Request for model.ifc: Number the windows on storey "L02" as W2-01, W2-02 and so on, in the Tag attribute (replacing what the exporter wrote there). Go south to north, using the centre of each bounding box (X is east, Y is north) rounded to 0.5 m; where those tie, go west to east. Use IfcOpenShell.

First a look at what the model holds.

```python
import ifcopenshell
import ifcopenshell.util.element
import ifcopenshell.util.placement

model = ifcopenshell.open("model.ifc")
print(model.schema)
storey = next(s for s in model.by_type("IfcBuildingStorey") if s.Name == "L02")
windows = [e for e in ifcopenshell.util.element.get_decomposition(storey) if e.is_a("IfcWindow")]
for e in sorted(windows, key=lambda e: e.id()):
    origin = ifcopenshell.util.placement.get_local_placement(e.ObjectPlacement)[:3, 3]
    print(e.id(), e.Tag, e.Name, origin.round(2) + 0.0, sep=" | ")
```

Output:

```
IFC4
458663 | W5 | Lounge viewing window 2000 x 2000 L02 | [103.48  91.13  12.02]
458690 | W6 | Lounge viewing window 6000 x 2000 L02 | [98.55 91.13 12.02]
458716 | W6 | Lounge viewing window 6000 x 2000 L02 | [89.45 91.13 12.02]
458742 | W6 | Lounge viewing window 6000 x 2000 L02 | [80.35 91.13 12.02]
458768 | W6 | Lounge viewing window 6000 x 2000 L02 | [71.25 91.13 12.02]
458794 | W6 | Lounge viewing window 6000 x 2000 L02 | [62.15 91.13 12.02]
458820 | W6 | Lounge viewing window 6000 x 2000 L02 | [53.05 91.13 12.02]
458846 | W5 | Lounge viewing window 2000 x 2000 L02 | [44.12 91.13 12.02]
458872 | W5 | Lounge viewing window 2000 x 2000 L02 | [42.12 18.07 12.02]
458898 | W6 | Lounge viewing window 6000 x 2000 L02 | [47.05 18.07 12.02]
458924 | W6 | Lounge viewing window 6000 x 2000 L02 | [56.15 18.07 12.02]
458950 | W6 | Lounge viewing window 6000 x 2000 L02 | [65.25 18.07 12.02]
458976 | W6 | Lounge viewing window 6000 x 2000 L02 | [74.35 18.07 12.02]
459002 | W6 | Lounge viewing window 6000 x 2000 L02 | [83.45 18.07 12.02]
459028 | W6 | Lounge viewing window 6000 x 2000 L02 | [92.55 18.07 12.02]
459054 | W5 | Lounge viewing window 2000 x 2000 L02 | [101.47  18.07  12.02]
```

```python
import ifcopenshell
import ifcopenshell.geom
import ifcopenshell.util.element
import ifcopenshell.util.shape

model = ifcopenshell.open("model.ifc")
settings = ifcopenshell.geom.settings()
settings.set("use-world-coords", True)


def centre(element):
    shape = ifcopenshell.geom.create_shape(settings, element)
    return ifcopenshell.util.shape.get_bbox_centroid(shape.geometry)


storey = next(s for s in model.by_type("IfcBuildingStorey") if s.Name == "L02")
windows = [e for e in ifcopenshell.util.element.get_decomposition(storey) if e.is_a("IfcWindow")]

# Insertion points can sit at a corner or the storey origin, so sort by the geometry (in metres).
centres = {e: centre(e) for e in windows}
windows.sort(key=lambda e: (round(centres[e][1] / 0.5), centres[e][0]))

for i, e in enumerate(windows, start=1):
    number = f"W2-{i:02d}"
    e.Tag = number
    print(e.id(), number)

model.write("model_v2.ifc")
```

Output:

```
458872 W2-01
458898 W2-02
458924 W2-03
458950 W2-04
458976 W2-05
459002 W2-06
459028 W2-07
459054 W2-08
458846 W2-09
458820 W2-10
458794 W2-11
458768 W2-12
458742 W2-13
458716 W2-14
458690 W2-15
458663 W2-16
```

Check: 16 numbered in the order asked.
